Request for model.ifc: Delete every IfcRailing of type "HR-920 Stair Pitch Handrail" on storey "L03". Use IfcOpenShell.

First a look at what the model holds.

```python
import ifcopenshell
import ifcopenshell.util.element

model = ifcopenshell.open("model.ifc")
print(model.schema)
storey = next(s for s in model.by_type("IfcBuildingStorey") if s.Name == "L03")
railings = [e for e in ifcopenshell.util.element.get_decomposition(storey) if e.is_a("IfcRailing")]
seen = {}
for e in railings:
    element_type = ifcopenshell.util.element.get_type(e)
    name = element_type.Name if element_type not in (None, e) else None
    seen[name] = seen.get(name, 0) + 1
for name, count in sorted(seen.items(), key=str):
    print(count, "x", name)
```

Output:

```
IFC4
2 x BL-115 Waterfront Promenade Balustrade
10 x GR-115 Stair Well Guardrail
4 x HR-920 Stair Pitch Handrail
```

```python
import ifcopenshell
import ifcopenshell.api.root
import ifcopenshell.util.element

model = ifcopenshell.open("model.ifc")

storey = next(s for s in model.by_type("IfcBuildingStorey") if s.Name == "L03")
railings = [e for e in ifcopenshell.util.element.get_decomposition(storey) if e.is_a("IfcRailing")]
targets = [e for e in railings if (t := ifcopenshell.util.element.get_type(e)) not in (None, e) and t.Name == "HR-920 Stair Pitch Handrail"]

for e in targets:
    ifcopenshell.api.root.remove_product(model, product=e)
print(len(targets), "removed")

model.write("model-out.ifc")
```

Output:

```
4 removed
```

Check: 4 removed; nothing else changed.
